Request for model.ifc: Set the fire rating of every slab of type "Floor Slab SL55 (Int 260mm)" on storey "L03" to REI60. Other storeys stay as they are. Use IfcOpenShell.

First a look at what the model holds.

```python
import ifcopenshell
import ifcopenshell.util.element

model = ifcopenshell.open("model.ifc")
print(model.schema)
storey = next(s for s in model.by_type("IfcBuildingStorey") if s.Name == "L03")
slabs = [e for e in ifcopenshell.util.element.get_decomposition(storey) if e.is_a("IfcSlab")]
seen = {}
for e in slabs:
    element_type = ifcopenshell.util.element.get_type(e)
    key = (element_type.Name if element_type != e and element_type else None, ifcopenshell.util.element.get_pset(e, "Pset_SlabCommon", "FireRating"))
    seen[key] = seen.get(key, 0) + 1
for (name, value), count in sorted(seen.items(), key=str):
    print(count, "x", name, "|", value)
```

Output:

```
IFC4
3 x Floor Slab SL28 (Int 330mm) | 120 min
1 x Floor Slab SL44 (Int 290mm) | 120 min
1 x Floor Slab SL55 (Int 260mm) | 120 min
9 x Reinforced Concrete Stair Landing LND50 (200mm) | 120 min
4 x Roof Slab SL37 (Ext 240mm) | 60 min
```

```python
import ifcopenshell
import ifcopenshell.api.pset
import ifcopenshell.util.element

model = ifcopenshell.open("model.ifc")

storey = next(s for s in model.by_type("IfcBuildingStorey") if s.Name == "L03")
slabs = [e for e in ifcopenshell.util.element.get_decomposition(storey) if e.is_a("IfcSlab")]

count = 0
for e in slabs:
    element_type = ifcopenshell.util.element.get_type(e)
    if element_type in (None, e) or element_type.Name != "Floor Slab SL55 (Int 260mm)":
        continue
    # add_pset returns the element's existing set when there is one.
    pset = ifcopenshell.api.pset.add_pset(model, product=e, name="Pset_SlabCommon")
    ifcopenshell.api.pset.edit_pset(model, pset=pset, properties={"FireRating": "REI60"})
    count += 1

print(count, "slabs updated")

model.write("model_rev.ifc")
```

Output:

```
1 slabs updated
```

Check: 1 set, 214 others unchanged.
